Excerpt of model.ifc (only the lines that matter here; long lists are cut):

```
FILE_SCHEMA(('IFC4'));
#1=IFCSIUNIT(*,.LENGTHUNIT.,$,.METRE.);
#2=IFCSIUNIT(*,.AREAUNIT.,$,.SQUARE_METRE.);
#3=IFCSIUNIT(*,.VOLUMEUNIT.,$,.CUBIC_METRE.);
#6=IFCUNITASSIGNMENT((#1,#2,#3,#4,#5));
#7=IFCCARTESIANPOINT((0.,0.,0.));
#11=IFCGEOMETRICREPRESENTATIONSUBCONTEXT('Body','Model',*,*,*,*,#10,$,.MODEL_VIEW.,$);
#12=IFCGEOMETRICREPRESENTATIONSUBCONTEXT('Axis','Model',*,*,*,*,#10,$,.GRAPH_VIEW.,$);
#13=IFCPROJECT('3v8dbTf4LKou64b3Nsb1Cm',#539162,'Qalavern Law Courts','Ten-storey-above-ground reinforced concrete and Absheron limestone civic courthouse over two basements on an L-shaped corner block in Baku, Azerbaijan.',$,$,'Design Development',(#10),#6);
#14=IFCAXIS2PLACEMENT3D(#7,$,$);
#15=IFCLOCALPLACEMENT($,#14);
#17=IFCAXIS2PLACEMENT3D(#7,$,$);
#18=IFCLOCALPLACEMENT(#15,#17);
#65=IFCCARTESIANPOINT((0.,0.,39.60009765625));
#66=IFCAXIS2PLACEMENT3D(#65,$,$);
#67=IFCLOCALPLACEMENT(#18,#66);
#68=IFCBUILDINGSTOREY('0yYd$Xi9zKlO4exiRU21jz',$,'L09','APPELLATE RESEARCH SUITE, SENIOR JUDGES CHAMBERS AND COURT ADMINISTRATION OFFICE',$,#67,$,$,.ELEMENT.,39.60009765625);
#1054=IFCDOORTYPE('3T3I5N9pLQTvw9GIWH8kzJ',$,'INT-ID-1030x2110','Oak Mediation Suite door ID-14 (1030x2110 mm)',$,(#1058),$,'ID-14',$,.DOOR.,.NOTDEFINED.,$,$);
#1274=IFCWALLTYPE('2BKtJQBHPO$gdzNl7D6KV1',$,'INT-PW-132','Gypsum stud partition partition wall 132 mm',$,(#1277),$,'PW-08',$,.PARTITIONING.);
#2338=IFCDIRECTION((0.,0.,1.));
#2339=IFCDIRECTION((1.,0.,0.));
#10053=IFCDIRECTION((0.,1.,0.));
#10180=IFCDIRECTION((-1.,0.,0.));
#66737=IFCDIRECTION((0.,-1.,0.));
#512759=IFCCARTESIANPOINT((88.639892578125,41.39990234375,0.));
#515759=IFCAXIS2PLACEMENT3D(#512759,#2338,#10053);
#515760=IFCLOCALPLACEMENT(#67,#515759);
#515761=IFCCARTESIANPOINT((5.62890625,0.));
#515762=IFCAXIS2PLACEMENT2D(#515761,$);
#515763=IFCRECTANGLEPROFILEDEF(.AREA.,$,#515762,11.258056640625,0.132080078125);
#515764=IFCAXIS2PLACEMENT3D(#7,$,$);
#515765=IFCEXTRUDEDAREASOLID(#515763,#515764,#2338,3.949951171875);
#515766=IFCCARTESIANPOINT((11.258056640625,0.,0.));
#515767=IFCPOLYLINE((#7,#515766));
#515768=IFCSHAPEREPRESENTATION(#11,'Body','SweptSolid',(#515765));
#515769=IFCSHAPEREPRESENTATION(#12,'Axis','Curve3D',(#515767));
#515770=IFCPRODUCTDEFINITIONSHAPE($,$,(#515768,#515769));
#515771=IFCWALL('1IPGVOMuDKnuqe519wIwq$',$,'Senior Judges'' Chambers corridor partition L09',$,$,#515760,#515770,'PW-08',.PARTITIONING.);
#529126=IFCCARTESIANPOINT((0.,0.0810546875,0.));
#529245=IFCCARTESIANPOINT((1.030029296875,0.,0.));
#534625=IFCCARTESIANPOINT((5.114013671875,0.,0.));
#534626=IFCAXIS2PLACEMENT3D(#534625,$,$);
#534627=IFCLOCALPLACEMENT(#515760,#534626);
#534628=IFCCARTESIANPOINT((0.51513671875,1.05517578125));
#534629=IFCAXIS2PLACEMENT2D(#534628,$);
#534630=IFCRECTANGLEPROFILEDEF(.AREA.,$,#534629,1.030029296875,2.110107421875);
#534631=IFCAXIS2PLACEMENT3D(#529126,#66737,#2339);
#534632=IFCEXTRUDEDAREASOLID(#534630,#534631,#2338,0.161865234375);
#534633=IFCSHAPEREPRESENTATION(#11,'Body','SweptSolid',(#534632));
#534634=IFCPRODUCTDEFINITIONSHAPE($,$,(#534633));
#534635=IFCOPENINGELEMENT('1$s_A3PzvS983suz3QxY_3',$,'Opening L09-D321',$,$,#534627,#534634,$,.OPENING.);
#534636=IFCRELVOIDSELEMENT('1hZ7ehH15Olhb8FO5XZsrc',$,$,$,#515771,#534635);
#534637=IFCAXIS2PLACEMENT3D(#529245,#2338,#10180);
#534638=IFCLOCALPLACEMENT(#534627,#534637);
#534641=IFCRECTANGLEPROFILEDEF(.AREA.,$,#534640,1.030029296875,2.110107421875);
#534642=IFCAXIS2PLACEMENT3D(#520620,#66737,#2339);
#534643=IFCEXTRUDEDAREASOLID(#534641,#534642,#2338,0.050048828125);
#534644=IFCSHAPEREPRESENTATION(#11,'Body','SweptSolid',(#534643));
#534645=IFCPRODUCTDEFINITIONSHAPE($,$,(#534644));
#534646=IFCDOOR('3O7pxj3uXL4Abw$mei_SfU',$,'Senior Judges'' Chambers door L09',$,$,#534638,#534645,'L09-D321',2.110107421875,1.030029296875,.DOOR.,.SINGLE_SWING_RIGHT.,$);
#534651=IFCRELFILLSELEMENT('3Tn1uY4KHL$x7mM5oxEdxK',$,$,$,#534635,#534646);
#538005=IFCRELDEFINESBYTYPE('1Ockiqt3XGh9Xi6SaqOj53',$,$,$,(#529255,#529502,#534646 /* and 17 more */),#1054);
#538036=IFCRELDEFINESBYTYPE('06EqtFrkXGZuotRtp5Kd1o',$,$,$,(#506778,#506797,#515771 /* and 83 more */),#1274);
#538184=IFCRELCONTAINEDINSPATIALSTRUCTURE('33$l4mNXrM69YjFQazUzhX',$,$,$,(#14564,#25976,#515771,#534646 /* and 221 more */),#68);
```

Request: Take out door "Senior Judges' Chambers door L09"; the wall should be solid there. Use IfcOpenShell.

```python
import ifcopenshell
import ifcopenshell.api.feature
import ifcopenshell.api.root
import ifcopenshell.geom
import ifcopenshell.util.shape

model = ifcopenshell.open("model.ifc")
settings = ifcopenshell.geom.settings()


def volume(element):
    """Net volume in cubic metres, openings subtracted."""
    shape = ifcopenshell.geom.create_shape(settings, element)
    return ifcopenshell.util.shape.get_volume(shape.geometry)


door = model.by_guid("3O7pxj3uXL4Abw$mei_SfU")
opening = door.FillsVoids[0].RelatingOpeningElement
wall = opening.VoidsElements[0].RelatingBuildingElement
before = volume(wall)

ifcopenshell.api.root.remove_product(model, product=door)
ifcopenshell.api.feature.remove_feature(model, feature=opening)

after = volume(wall)

print(f"wall volume {before:.3f} -> {after:.3f} m3")

model.write("model_updated.ifc")
```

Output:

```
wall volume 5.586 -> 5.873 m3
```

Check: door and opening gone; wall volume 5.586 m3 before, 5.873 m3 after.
